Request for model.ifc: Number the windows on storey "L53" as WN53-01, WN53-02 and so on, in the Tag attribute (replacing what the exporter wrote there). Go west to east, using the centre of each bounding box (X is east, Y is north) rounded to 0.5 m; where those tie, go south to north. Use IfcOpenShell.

First a look at what the model holds.

```python
import ifcopenshell
import ifcopenshell.util.element
import ifcopenshell.util.placement

model = ifcopenshell.open("model.ifc")
print(model.schema)
storey = next(s for s in model.by_type("IfcBuildingStorey") if s.Name == "L53")
windows = [e for e in ifcopenshell.util.element.get_decomposition(storey) if e.is_a("IfcWindow")]
for e in sorted(windows, key=lambda e: e.id()):
    origin = ifcopenshell.util.placement.get_local_placement(e.ObjectPlacement)[:3, 3]
    print(e.id(), e.Tag, e.Name, origin.round(2) + 0.0, sep=" | ")
```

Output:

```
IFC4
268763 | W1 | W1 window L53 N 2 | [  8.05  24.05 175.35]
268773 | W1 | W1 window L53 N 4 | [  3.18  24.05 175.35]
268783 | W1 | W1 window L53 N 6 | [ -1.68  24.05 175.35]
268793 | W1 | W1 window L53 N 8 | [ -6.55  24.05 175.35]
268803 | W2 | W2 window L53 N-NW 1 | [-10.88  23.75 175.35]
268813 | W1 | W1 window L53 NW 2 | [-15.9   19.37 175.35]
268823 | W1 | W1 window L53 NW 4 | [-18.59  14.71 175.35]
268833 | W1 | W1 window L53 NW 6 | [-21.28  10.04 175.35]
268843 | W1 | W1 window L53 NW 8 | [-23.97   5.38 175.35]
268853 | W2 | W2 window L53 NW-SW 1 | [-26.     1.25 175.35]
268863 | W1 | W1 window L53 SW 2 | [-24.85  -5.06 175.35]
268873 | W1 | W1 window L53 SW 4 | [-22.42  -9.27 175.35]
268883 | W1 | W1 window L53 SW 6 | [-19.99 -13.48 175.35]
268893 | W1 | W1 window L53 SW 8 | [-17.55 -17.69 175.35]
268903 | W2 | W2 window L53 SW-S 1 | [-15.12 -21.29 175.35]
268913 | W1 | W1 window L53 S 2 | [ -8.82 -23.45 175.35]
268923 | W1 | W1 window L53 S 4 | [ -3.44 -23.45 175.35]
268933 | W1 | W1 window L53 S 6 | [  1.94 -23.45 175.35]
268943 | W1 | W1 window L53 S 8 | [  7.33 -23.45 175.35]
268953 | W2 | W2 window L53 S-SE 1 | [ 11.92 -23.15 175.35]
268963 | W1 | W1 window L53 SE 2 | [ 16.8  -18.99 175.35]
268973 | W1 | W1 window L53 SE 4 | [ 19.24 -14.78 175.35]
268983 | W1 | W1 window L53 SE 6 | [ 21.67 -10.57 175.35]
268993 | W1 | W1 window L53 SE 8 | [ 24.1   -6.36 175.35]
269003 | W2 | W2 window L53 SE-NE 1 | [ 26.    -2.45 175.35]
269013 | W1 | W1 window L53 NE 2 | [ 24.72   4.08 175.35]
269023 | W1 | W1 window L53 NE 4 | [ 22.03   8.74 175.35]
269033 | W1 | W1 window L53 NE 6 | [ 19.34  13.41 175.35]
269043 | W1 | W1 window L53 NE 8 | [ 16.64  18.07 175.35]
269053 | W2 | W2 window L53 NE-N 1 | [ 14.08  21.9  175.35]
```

```python
import ifcopenshell
import ifcopenshell.geom
import ifcopenshell.util.element
import ifcopenshell.util.shape

model = ifcopenshell.open("model.ifc")
settings = ifcopenshell.geom.settings()
settings.set("use-world-coords", True)


def centre(element):
    shape = ifcopenshell.geom.create_shape(settings, element)
    return ifcopenshell.util.shape.get_bbox_centroid(shape.geometry)


storey = next(s for s in model.by_type("IfcBuildingStorey") if s.Name == "L53")
windows = [e for e in ifcopenshell.util.element.get_decomposition(storey) if e.is_a("IfcWindow")]

# Insertion points can sit at a corner or the storey origin, so sort by the geometry (in metres).
centres = {e: centre(e) for e in windows}
windows.sort(key=lambda e: (round(centres[e][0] / 0.5), centres[e][1]))

for i, e in enumerate(windows, start=1):
    number = f"WN53-{i:02d}"
    e.Tag = number
    print(e.id(), number)

model.write("model-out.ifc")
```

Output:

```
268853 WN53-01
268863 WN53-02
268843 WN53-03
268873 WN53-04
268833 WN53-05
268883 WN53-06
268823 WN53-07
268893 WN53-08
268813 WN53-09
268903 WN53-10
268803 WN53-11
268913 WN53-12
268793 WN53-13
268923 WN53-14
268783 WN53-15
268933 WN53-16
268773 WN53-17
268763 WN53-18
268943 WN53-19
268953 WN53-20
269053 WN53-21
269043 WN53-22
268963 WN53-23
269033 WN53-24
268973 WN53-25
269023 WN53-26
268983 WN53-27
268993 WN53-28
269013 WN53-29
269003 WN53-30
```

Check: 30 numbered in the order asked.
